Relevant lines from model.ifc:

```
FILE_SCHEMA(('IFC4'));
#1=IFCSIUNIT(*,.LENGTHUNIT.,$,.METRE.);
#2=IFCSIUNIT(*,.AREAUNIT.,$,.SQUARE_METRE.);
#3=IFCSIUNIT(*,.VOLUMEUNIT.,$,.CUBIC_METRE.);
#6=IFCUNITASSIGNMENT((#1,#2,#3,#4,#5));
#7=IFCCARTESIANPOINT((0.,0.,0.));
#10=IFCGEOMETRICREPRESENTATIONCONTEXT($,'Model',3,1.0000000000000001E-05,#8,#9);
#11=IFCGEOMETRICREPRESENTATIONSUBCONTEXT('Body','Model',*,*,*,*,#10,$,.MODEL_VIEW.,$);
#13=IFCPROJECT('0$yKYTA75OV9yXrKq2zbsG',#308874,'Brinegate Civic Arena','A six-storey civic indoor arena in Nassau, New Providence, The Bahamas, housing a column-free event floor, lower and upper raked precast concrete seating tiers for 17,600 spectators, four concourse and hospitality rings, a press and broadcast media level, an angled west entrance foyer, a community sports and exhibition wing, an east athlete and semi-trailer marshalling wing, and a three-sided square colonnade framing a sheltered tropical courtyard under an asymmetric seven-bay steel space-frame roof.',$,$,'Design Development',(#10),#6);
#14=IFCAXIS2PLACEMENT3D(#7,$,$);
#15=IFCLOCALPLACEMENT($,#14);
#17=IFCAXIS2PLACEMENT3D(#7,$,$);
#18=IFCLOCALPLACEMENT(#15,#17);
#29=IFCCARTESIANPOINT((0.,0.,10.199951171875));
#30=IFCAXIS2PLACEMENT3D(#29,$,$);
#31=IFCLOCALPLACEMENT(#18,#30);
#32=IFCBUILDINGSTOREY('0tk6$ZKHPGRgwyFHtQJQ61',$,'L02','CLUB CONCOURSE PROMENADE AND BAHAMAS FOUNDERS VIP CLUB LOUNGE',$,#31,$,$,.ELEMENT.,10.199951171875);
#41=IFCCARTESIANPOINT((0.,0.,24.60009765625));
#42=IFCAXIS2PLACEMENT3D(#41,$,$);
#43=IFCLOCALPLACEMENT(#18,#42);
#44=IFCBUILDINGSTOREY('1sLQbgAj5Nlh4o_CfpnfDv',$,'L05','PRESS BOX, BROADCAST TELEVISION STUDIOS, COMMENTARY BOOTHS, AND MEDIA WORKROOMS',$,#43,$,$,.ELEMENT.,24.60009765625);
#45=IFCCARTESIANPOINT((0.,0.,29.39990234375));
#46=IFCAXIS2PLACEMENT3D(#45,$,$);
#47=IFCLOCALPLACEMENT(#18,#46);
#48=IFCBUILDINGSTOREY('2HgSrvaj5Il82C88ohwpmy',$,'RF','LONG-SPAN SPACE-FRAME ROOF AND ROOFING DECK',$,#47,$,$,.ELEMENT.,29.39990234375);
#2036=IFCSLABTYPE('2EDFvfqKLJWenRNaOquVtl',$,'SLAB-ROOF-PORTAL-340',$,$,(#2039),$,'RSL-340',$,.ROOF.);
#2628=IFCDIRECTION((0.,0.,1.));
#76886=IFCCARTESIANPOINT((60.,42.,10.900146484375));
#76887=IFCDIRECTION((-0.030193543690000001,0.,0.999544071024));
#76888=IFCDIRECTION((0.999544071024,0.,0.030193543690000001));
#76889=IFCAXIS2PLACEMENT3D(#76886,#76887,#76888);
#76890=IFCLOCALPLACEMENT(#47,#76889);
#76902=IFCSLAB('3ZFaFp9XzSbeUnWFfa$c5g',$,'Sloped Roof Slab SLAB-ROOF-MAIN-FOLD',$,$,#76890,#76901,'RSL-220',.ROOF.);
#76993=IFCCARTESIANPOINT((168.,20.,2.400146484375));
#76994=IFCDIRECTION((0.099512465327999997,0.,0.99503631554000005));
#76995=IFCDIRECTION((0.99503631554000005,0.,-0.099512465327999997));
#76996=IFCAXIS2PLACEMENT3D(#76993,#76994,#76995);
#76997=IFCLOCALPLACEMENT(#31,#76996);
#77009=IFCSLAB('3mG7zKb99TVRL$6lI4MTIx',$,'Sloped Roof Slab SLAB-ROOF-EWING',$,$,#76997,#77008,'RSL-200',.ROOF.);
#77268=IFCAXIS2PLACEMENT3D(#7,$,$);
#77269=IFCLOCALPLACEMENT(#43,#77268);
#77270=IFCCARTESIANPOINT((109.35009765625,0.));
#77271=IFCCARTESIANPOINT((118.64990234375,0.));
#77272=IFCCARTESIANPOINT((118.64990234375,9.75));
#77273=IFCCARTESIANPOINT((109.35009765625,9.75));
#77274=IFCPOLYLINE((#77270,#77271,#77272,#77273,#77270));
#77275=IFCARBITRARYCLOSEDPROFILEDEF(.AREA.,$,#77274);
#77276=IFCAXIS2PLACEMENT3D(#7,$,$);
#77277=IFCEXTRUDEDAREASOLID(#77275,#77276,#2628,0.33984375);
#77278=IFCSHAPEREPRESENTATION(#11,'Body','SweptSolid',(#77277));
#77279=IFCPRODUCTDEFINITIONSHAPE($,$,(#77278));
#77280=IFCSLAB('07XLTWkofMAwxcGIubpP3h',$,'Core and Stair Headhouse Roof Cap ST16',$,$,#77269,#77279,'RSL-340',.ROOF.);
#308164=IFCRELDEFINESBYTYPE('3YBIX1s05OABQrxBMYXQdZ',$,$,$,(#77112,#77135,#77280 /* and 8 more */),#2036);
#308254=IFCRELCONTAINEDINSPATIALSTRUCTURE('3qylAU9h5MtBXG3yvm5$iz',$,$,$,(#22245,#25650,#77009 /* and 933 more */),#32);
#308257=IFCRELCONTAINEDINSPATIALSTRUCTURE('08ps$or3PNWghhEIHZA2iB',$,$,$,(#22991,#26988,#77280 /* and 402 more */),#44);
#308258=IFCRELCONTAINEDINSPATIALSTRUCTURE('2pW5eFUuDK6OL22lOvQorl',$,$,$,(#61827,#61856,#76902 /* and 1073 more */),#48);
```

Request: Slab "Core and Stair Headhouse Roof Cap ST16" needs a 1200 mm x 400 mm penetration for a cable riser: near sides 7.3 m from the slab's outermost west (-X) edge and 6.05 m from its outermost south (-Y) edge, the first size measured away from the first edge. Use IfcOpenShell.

```python
import numpy as np
import ifcopenshell
import ifcopenshell.api.feature
import ifcopenshell.api.geometry
import ifcopenshell.api.root
import ifcopenshell.geom
import ifcopenshell.util.placement
import ifcopenshell.util.representation
import ifcopenshell.util.shape
import ifcopenshell.util.unit

model = ifcopenshell.open("model.ifc")
unit_scale = ifcopenshell.util.unit.calculate_unit_scale(model)
settings = ifcopenshell.geom.settings()


def volume(element):
    """Net volume in cubic metres, openings subtracted."""
    shape = ifcopenshell.geom.create_shape(settings, element)
    return ifcopenshell.util.shape.get_volume(shape.geometry)


slab = model.by_guid("07XLTWkofMAwxcGIubpP3h")
before = volume(slab)

# Extent in the slab's own axes, in metres. The edges named are its -X and -Y sides.
slab_shape = ifcopenshell.geom.create_shape(settings, slab)
vertices = ifcopenshell.util.shape.get_vertices(slab_shape.geometry)
x_min, y_min, bottom = vertices.min(axis=0)
top = vertices[:, 2].max()

opening = ifcopenshell.api.root.create_entity(model, ifc_class="IfcOpeningElement", name="Cable riser opening", predefined_type="OPENING")
context = ifcopenshell.util.representation.get_context(model, "Model", "Body", "MODEL_VIEW")
width, depth = 1.2, 0.4
outline = [(0.0, 0.0), (width, 0.0), (width, depth), (0.0, depth), (0.0, 0.0)]
# Overshoot both faces by 50 mm so the cut is clean.
shape = ifcopenshell.api.geometry.add_slab_representation(
    model, context=context, depth=top - bottom + 0.1, polyline=outline
)
ifcopenshell.api.geometry.assign_representation(model, product=opening, representation=shape)

matrix = ifcopenshell.util.placement.get_local_placement(slab.ObjectPlacement)
matrix[:, 3] = matrix @ np.append(np.array([x_min + 7.3, y_min + 6.05, bottom - 0.05]) / unit_scale, 1.0)
ifcopenshell.api.geometry.edit_object_placement(model, product=opening, matrix=matrix, is_si=False)
ifcopenshell.api.feature.add_feature(model, feature=opening, element=slab)

after = volume(slab)

print(f"slab volume {before:.3f} -> {after:.3f} m3")

model.write("model_edited.ifc")
```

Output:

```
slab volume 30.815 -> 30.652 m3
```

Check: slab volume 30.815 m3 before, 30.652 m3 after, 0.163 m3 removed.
